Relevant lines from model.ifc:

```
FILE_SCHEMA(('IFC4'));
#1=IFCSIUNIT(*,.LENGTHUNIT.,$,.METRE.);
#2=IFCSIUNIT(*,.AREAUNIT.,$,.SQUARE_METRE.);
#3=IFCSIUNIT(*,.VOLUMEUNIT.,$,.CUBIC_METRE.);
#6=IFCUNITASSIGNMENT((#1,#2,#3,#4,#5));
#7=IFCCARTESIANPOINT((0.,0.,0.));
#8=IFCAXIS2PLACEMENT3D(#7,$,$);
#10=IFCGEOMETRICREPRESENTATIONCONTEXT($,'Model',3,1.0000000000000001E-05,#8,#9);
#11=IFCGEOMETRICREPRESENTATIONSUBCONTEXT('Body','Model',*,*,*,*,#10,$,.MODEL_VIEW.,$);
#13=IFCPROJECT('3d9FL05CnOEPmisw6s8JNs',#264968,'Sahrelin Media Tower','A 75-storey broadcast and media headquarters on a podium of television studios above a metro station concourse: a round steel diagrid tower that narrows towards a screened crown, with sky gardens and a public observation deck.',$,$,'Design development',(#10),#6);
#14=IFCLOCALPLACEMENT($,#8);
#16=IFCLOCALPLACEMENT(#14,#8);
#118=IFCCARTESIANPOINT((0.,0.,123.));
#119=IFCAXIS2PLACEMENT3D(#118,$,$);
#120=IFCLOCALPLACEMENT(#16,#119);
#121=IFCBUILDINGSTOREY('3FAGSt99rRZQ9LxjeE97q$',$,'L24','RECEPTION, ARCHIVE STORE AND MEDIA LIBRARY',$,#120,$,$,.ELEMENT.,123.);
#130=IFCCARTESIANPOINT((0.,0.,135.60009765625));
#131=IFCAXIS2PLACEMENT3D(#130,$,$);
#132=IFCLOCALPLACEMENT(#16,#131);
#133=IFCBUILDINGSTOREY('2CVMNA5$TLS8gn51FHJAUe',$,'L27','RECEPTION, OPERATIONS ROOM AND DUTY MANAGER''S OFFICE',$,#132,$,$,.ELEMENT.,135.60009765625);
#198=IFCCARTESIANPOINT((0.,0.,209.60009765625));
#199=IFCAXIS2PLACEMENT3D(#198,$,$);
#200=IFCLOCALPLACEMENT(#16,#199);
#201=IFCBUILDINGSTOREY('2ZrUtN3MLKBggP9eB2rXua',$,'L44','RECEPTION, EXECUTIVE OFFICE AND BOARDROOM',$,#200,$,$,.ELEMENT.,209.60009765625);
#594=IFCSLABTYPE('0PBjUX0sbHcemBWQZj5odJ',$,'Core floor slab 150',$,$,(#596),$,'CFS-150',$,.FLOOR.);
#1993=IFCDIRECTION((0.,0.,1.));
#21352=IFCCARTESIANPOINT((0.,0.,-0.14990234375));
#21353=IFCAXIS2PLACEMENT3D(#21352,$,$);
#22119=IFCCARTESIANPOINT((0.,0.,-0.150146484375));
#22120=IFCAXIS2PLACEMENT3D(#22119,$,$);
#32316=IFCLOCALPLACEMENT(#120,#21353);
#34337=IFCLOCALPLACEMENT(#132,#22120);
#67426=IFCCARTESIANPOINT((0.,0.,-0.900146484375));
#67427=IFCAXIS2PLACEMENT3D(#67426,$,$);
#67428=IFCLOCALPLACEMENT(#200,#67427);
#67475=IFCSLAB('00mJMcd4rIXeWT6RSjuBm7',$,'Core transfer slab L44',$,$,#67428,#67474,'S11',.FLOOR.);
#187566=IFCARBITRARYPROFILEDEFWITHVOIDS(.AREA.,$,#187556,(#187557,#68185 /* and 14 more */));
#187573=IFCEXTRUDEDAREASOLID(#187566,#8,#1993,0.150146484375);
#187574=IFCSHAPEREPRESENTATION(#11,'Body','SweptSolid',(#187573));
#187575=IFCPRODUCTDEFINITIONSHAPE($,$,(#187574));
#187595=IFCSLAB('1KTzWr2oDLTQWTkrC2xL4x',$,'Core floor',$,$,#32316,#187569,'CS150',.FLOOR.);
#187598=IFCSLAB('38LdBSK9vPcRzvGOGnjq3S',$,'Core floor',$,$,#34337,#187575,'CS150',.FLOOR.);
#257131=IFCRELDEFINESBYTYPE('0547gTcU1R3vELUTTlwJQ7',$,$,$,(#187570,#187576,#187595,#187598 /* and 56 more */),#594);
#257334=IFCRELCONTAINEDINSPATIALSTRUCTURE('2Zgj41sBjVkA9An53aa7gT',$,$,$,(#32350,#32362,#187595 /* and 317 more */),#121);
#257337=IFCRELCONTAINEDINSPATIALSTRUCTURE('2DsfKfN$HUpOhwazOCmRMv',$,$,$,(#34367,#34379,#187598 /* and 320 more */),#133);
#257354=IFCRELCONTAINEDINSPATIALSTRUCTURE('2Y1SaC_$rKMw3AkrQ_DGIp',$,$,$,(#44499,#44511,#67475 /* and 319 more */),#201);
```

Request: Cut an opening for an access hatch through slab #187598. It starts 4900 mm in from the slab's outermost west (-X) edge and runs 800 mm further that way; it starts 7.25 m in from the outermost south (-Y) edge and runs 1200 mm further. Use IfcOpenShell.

```python
import numpy as np
import ifcopenshell
import ifcopenshell.api.feature
import ifcopenshell.api.geometry
import ifcopenshell.api.root
import ifcopenshell.geom
import ifcopenshell.util.placement
import ifcopenshell.util.representation
import ifcopenshell.util.shape
import ifcopenshell.util.unit

model = ifcopenshell.open("model.ifc")
unit_scale = ifcopenshell.util.unit.calculate_unit_scale(model)
settings = ifcopenshell.geom.settings()


def volume(element):
    """Net volume in cubic metres, openings subtracted."""
    shape = ifcopenshell.geom.create_shape(settings, element)
    return ifcopenshell.util.shape.get_volume(shape.geometry)


slab = model.by_id(187598)
before = volume(slab)

# Extent in the slab's own axes, in metres. The edges named are its -X and -Y sides.
slab_shape = ifcopenshell.geom.create_shape(settings, slab)
vertices = ifcopenshell.util.shape.get_vertices(slab_shape.geometry)
x_min, y_min, bottom = vertices.min(axis=0)
top = vertices[:, 2].max()

opening = ifcopenshell.api.root.create_entity(model, ifc_class="IfcOpeningElement", name="Access hatch opening", predefined_type="OPENING")
context = ifcopenshell.util.representation.get_context(model, "Model", "Body", "MODEL_VIEW")
width, depth = 0.8, 1.2
outline = [(0.0, 0.0), (width, 0.0), (width, depth), (0.0, depth), (0.0, 0.0)]
# Overshoot both faces by 50 mm so the cut is clean.
shape = ifcopenshell.api.geometry.add_slab_representation(
    model, context=context, depth=top - bottom + 0.1, polyline=outline
)
ifcopenshell.api.geometry.assign_representation(model, product=opening, representation=shape)

matrix = ifcopenshell.util.placement.get_local_placement(slab.ObjectPlacement)
matrix[:, 3] = matrix @ np.append(np.array([x_min + 4.9, y_min + 7.25, bottom - 0.05]) / unit_scale, 1.0)
ifcopenshell.api.geometry.edit_object_placement(model, product=opening, matrix=matrix, is_si=False)
ifcopenshell.api.feature.add_feature(model, feature=opening, element=slab)

after = volume(slab)

print(f"slab volume {before:.3f} -> {after:.3f} m3")

model.write("model_edited.ifc")
```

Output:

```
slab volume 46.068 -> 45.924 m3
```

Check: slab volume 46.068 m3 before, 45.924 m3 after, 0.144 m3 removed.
